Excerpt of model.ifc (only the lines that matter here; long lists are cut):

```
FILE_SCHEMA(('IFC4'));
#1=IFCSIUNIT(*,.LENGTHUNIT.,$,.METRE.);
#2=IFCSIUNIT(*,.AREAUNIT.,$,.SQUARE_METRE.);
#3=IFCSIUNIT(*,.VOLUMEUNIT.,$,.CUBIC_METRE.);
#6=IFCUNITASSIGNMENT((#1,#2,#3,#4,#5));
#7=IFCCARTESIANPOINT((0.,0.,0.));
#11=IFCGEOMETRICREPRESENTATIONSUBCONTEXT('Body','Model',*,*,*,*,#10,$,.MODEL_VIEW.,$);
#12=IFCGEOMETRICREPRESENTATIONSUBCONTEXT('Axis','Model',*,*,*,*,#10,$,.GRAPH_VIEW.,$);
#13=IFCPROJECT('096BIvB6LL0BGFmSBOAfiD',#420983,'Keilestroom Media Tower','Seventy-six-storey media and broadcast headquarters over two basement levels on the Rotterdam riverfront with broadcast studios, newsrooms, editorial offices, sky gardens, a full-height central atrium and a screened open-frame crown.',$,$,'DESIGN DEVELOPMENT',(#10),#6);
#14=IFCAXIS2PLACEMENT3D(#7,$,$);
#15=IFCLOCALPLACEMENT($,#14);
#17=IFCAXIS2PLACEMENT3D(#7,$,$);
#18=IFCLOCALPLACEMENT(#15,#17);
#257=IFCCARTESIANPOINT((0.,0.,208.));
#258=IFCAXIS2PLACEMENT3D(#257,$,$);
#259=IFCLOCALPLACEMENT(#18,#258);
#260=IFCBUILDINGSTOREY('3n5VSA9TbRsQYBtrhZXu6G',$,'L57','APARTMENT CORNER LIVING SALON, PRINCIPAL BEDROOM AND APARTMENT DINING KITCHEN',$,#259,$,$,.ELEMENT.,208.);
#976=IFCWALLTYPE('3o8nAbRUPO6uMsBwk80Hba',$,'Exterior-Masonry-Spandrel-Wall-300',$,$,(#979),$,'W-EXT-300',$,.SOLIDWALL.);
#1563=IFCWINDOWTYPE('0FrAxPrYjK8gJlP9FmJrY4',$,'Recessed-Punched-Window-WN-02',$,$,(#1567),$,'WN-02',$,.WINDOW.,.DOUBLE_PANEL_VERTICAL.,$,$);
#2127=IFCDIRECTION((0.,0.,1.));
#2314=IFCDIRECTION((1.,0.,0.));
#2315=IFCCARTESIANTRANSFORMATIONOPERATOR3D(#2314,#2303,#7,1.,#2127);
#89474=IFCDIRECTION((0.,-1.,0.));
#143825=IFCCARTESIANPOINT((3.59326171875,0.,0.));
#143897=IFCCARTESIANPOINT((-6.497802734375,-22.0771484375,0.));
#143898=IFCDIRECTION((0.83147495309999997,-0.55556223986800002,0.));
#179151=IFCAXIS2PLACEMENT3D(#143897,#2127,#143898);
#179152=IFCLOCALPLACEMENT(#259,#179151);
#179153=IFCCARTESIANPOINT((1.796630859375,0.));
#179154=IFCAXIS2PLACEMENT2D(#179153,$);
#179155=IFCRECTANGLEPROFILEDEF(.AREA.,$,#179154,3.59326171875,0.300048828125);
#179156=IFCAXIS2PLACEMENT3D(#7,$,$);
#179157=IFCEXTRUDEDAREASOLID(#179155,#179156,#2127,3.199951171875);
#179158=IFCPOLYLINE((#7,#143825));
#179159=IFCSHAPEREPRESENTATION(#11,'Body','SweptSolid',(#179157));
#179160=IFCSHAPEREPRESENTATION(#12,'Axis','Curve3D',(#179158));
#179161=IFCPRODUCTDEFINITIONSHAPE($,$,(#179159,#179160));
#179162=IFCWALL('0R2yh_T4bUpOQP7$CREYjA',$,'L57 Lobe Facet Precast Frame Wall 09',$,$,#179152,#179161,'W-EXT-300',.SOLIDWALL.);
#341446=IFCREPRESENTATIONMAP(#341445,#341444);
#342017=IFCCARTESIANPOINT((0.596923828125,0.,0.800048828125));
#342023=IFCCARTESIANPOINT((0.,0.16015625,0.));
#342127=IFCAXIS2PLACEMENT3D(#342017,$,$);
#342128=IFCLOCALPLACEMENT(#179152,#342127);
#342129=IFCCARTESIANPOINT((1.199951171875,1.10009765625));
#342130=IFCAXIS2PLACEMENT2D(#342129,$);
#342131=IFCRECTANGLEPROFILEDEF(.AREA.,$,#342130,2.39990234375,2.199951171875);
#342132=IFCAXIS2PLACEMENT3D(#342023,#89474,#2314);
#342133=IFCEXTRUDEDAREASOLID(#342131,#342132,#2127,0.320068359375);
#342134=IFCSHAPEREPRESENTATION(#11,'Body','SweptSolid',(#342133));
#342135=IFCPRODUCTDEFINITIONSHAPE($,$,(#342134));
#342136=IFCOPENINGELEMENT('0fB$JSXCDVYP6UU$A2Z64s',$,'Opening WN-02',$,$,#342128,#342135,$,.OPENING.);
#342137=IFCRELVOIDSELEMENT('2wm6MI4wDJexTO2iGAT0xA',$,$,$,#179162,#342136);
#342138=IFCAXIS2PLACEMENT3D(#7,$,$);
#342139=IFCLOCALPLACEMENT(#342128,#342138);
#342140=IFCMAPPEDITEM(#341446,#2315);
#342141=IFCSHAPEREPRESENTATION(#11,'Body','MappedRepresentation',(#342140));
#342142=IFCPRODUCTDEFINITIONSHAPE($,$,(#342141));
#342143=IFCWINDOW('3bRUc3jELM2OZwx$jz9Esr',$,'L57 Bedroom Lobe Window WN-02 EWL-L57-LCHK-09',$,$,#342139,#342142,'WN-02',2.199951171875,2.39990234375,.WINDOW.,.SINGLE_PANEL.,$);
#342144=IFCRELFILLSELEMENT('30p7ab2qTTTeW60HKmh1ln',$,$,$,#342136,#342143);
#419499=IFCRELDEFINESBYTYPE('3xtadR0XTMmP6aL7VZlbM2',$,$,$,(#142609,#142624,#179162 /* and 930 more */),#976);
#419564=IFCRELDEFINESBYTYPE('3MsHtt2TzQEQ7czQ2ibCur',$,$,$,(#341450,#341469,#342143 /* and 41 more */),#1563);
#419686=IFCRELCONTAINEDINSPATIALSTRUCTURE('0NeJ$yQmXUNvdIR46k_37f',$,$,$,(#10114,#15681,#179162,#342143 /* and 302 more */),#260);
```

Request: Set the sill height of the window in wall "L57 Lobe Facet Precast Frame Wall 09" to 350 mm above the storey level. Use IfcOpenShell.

```python
import numpy as np
import ifcopenshell
import ifcopenshell.api.geometry
import ifcopenshell.geom
import ifcopenshell.util.element
import ifcopenshell.util.placement
import ifcopenshell.util.shape
import ifcopenshell.util.unit

model = ifcopenshell.open("model.ifc")
unit_scale = ifcopenshell.util.unit.calculate_unit_scale(model)

window = model.by_guid("3bRUc3jELM2OZwx$jz9Esr")
opening = window.FillsVoids[0].RelatingOpeningElement
storey = ifcopenshell.util.element.get_container(window, ifc_class="IfcBuildingStorey")
level = ifcopenshell.util.placement.get_local_placement(storey.ObjectPlacement)[2, 3]

# The opening's origin need not be at the sill, so measure its lowest point.
shape = ifcopenshell.geom.create_shape(ifcopenshell.geom.settings(), opening)
bottom = ifcopenshell.util.shape.get_shape_bottom_elevation(shape, shape.geometry) / unit_scale
dz = level + 0.35 / unit_scale - bottom

shift = np.array([0.0, 0.0, dz])
# The window is placed relative to its opening, so it follows when the opening moves.
matrix = ifcopenshell.util.placement.get_local_placement(opening.ObjectPlacement)
matrix[:3, 3] += shift
ifcopenshell.api.geometry.edit_object_placement(
    model, product=opening, matrix=matrix, is_si=False, should_transform_children=True
)

print(f"moved by {dz * unit_scale:+.3f} m")

model.write("model_v2.ifc")
```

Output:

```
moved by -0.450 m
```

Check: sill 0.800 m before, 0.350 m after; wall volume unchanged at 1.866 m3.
